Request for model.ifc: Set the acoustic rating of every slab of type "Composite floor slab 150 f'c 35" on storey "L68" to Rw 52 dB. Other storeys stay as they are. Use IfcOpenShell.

First a look at what the model holds.

```python
import ifcopenshell
import ifcopenshell.util.element

model = ifcopenshell.open("model.ifc")
print(model.schema)
storey = next(s for s in model.by_type("IfcBuildingStorey") if s.Name == "L68")
slabs = [e for e in ifcopenshell.util.element.get_decomposition(storey) if e.is_a("IfcSlab")]
seen = {}
for e in slabs:
    element_type = ifcopenshell.util.element.get_type(e)
    key = (element_type.Name if element_type != e and element_type else None, ifcopenshell.util.element.get_pset(e, "Pset_SlabCommon", "AcousticRating"))
    seen[key] = seen.get(key, 0) + 1
for (name, value), count in sorted(seen.items(), key=str):
    print(count, "x", name, "|", value)
```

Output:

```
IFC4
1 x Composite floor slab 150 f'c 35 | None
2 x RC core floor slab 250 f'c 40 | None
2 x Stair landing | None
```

```python
import ifcopenshell
import ifcopenshell.api.pset
import ifcopenshell.util.element

model = ifcopenshell.open("model.ifc")

storey = next(s for s in model.by_type("IfcBuildingStorey") if s.Name == "L68")
slabs = [e for e in ifcopenshell.util.element.get_decomposition(storey) if e.is_a("IfcSlab")]

count = 0
for e in slabs:
    element_type = ifcopenshell.util.element.get_type(e)
    if element_type in (None, e) or element_type.Name != "Composite floor slab 150 f'c 35":
        continue
    found = ifcopenshell.util.element.get_pset(e, "Pset_SlabCommon", should_inherit=False)
    if found:
        pset = model.by_id(found["id"])
        if len(ifcopenshell.util.element.get_elements_by_pset(pset)) > 1:
            pset = ifcopenshell.api.pset.unshare_pset(model, products=[e], pset=pset)[0]
    else:
        pset = ifcopenshell.api.pset.add_pset(model, product=e, name="Pset_SlabCommon")
    ifcopenshell.api.pset.edit_pset(model, pset=pset, properties={"AcousticRating": "Rw 52 dB"})
    count += 1

print(count, "slabs updated")

model.write("model_edited.ifc")
```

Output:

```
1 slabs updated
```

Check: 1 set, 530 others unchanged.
